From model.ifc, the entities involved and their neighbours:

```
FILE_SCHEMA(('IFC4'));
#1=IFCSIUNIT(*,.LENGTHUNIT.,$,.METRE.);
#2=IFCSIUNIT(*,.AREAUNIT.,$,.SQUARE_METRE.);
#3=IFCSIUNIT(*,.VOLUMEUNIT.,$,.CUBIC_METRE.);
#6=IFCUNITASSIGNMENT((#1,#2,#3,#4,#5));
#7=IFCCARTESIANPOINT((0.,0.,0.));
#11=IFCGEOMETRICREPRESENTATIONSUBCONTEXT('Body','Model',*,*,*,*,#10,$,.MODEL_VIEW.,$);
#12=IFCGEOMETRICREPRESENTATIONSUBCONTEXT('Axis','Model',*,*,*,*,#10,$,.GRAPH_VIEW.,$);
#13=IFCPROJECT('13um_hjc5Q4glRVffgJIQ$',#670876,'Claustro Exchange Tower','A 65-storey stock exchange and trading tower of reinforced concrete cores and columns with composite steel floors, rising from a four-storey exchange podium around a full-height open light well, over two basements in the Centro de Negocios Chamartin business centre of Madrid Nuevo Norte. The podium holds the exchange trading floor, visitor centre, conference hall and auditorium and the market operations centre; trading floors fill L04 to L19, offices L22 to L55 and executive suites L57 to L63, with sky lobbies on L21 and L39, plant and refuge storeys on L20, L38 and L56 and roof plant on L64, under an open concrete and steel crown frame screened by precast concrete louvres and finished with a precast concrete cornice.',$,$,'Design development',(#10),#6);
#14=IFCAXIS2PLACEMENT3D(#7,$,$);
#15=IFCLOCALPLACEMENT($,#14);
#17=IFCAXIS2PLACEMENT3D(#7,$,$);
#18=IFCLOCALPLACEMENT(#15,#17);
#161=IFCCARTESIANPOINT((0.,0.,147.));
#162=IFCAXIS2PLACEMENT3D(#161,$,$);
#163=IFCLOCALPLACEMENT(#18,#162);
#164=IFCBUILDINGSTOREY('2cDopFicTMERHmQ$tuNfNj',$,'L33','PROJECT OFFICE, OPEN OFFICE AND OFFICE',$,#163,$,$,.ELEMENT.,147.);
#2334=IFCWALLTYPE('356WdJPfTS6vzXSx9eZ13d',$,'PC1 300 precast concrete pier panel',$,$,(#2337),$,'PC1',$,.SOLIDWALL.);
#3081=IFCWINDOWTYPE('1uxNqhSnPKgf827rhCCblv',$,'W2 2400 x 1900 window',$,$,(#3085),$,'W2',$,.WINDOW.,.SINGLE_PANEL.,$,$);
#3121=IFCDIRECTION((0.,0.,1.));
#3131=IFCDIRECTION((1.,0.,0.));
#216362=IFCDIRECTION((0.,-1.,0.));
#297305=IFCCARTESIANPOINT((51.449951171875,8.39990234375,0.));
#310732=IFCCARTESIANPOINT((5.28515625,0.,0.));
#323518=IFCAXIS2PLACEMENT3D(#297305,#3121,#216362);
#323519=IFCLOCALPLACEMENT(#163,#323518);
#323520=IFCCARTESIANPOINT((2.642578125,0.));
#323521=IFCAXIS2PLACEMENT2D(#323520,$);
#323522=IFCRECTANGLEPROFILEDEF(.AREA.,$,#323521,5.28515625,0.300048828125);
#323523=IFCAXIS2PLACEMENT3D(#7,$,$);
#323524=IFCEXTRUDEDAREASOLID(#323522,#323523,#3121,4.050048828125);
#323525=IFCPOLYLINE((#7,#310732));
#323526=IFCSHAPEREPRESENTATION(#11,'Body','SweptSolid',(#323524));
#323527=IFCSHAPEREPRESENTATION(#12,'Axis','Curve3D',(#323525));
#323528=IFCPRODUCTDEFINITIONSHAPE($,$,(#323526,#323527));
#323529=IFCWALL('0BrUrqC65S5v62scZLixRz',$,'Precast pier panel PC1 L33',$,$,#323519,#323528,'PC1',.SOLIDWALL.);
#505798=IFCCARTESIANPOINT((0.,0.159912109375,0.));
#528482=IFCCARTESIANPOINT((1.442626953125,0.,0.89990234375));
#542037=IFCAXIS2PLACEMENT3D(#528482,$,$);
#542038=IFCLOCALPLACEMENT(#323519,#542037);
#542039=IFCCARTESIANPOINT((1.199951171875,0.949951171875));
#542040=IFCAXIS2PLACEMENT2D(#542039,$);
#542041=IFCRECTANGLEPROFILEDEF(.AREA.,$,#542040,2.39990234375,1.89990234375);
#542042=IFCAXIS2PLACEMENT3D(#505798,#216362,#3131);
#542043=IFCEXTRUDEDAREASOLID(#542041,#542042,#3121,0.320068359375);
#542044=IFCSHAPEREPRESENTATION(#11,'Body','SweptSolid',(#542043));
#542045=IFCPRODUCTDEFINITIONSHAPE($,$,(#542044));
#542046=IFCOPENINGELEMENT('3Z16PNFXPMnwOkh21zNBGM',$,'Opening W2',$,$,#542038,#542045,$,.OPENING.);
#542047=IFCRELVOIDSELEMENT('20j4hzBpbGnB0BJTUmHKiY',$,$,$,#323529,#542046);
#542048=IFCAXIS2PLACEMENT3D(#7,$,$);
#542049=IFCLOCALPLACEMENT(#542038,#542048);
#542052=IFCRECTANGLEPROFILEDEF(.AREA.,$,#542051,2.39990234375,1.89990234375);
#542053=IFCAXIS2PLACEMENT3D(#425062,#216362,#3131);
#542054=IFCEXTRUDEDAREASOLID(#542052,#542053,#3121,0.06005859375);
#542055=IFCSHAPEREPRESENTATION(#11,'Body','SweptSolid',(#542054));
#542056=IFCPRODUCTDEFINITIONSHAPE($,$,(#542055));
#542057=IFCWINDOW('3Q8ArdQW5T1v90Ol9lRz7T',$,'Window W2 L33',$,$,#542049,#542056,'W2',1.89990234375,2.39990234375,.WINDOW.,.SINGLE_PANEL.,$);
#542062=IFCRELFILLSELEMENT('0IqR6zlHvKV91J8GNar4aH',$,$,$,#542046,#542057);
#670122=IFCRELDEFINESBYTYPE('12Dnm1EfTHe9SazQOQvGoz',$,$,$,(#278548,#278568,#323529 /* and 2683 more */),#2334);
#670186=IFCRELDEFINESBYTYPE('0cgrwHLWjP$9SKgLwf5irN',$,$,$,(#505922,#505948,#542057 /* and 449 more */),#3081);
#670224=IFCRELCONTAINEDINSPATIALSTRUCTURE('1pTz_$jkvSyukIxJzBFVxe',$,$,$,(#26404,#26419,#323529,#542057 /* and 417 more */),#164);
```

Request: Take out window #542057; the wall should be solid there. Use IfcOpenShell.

```python
import ifcopenshell
import ifcopenshell.api.feature
import ifcopenshell.api.root
import ifcopenshell.geom
import ifcopenshell.util.shape

model = ifcopenshell.open("model.ifc")
settings = ifcopenshell.geom.settings()


def volume(element):
    """Net volume in cubic metres, openings subtracted."""
    shape = ifcopenshell.geom.create_shape(settings, element)
    return ifcopenshell.util.shape.get_volume(shape.geometry)


window = model.by_guid("3Q8ArdQW5T1v90Ol9lRz7T")
opening = window.FillsVoids[0].RelatingOpeningElement
wall = opening.VoidsElements[0].RelatingBuildingElement
before = volume(wall)

ifcopenshell.api.root.remove_product(model, product=window)
ifcopenshell.api.feature.remove_feature(model, feature=opening)

after = volume(wall)

print(f"wall volume {before:.3f} -> {after:.3f} m3")

model.write("model_v2.ifc")
```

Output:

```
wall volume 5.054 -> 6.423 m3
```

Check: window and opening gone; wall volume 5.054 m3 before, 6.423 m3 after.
